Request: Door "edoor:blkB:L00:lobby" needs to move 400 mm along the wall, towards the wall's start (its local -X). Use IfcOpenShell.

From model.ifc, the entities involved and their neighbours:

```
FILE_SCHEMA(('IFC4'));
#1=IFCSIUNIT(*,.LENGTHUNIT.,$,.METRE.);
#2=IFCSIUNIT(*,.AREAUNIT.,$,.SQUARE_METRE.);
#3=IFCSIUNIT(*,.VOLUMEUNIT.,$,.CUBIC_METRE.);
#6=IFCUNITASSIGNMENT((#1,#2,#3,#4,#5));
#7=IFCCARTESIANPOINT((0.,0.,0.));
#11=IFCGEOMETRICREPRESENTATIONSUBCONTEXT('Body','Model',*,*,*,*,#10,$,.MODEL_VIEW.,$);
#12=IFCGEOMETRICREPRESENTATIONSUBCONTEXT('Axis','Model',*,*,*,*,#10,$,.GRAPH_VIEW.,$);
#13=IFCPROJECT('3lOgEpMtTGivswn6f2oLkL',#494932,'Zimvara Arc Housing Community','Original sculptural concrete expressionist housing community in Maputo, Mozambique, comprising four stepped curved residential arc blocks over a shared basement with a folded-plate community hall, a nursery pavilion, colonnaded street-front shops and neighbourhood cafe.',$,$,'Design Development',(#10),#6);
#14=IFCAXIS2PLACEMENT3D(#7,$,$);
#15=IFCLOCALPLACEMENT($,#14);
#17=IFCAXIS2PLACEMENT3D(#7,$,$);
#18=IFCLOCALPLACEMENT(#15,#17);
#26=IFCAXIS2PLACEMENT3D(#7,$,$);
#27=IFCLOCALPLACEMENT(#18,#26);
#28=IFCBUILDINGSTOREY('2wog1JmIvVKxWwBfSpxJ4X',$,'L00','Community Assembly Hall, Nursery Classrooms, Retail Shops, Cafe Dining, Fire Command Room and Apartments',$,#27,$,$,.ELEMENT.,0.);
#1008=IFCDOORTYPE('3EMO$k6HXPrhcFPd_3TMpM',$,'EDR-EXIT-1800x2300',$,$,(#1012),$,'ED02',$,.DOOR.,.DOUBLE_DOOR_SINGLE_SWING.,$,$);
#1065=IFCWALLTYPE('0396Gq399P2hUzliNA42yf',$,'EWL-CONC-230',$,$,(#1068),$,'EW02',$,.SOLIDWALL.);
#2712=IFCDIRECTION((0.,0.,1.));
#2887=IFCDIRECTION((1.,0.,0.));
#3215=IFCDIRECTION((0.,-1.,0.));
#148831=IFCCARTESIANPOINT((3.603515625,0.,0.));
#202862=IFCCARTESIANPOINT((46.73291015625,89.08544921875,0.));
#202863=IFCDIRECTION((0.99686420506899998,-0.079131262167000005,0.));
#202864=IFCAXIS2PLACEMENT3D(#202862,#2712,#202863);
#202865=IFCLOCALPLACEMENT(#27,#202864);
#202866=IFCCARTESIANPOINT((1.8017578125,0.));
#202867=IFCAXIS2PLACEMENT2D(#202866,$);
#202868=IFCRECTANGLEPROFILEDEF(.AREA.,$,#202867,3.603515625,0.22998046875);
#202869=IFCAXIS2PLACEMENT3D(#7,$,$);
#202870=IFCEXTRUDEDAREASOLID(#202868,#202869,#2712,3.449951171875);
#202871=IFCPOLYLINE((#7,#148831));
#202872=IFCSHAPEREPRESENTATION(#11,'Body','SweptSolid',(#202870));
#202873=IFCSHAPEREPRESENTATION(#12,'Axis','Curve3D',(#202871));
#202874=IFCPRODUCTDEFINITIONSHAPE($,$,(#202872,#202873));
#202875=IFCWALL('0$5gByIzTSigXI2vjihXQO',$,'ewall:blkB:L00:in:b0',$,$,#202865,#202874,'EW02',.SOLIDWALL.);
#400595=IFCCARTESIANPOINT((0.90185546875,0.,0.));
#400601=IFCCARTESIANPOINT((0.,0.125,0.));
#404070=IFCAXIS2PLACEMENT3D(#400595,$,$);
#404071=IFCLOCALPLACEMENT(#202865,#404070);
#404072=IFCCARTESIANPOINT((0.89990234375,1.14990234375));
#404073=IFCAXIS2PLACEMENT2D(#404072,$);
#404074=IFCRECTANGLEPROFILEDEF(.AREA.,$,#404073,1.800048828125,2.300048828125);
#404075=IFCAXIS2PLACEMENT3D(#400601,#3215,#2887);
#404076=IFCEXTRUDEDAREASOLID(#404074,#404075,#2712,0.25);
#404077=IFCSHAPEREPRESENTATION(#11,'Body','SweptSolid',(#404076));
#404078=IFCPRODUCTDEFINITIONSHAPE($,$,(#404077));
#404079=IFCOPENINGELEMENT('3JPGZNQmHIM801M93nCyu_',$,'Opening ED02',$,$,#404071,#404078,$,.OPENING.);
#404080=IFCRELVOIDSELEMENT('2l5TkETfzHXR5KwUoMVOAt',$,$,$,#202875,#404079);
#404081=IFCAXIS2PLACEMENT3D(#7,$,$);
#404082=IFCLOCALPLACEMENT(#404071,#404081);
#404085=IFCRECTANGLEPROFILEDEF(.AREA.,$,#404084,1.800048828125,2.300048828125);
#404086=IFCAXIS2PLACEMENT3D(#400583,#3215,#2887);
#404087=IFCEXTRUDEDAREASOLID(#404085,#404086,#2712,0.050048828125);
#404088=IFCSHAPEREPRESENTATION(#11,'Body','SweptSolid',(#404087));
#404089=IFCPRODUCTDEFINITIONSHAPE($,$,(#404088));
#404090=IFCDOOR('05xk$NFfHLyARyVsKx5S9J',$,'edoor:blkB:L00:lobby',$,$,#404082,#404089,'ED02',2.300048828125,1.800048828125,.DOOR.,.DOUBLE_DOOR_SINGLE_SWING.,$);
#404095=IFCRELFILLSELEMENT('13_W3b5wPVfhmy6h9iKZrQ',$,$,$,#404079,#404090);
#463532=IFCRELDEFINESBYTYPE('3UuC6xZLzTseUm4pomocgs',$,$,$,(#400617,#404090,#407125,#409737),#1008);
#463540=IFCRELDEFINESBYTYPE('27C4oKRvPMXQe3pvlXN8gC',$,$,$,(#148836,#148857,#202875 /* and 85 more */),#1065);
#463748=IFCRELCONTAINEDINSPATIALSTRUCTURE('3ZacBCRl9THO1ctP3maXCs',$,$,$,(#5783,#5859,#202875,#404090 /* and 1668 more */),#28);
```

```python
import ifcopenshell
import ifcopenshell.api.geometry
import ifcopenshell.util.placement

model = ifcopenshell.open("model.ifc")

door = model.by_guid("05xk$NFfHLyARyVsKx5S9J")
opening = door.FillsVoids[0].RelatingOpeningElement
wall = opening.VoidsElements[0].RelatingBuildingElement

wall_matrix = ifcopenshell.util.placement.get_local_placement(wall.ObjectPlacement)
shift = wall_matrix[:3, 0] * -0.4
before = ifcopenshell.util.placement.get_local_placement(door.ObjectPlacement)[:3, 3].copy()

# The door is placed relative to its opening, so it follows when the opening moves.
matrix = ifcopenshell.util.placement.get_local_placement(opening.ObjectPlacement)
matrix[:3, 3] += shift
ifcopenshell.api.geometry.edit_object_placement(
    model, product=opening, matrix=matrix, is_si=False, should_transform_children=True
)

after = ifcopenshell.util.placement.get_local_placement(door.ObjectPlacement)[:3, 3]
print("door moved by", (after - before).round(3) + 0.0)

model.write("model_rev.ifc")
```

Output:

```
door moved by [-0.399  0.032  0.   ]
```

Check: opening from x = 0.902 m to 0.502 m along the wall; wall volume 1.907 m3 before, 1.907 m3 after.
